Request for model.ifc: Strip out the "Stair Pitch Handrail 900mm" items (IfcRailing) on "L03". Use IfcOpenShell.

First a look at what the model holds.

```python
import ifcopenshell
import ifcopenshell.util.element

model = ifcopenshell.open("model.ifc")
print(model.schema)
storey = next(s for s in model.by_type("IfcBuildingStorey") if s.Name == "L03")
railings = [e for e in ifcopenshell.util.element.get_decomposition(storey) if e.is_a("IfcRailing")]
seen = {}
for e in railings:
    element_type = ifcopenshell.util.element.get_type(e)
    name = element_type.Name if element_type not in (None, e) else None
    seen[name] = seen.get(name, 0) + 1
for name, count in sorted(seen.items(), key=str):
    print(count, "x", name)
```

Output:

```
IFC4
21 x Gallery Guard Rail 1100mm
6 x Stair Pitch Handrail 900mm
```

```python
import ifcopenshell
import ifcopenshell.api.root
import ifcopenshell.util.element

model = ifcopenshell.open("model.ifc")

storey = next(s for s in model.by_type("IfcBuildingStorey") if s.Name == "L03")
railings = [e for e in ifcopenshell.util.element.get_decomposition(storey) if e.is_a("IfcRailing")]
targets = [e for e in railings if (t := ifcopenshell.util.element.get_type(e)) not in (None, e) and t.Name == "Stair Pitch Handrail 900mm"]

for e in targets:
    ifcopenshell.api.root.remove_product(model, product=e)
print(len(targets), "removed")

model.write("model_rev.ifc")
```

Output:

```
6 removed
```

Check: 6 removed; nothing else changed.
